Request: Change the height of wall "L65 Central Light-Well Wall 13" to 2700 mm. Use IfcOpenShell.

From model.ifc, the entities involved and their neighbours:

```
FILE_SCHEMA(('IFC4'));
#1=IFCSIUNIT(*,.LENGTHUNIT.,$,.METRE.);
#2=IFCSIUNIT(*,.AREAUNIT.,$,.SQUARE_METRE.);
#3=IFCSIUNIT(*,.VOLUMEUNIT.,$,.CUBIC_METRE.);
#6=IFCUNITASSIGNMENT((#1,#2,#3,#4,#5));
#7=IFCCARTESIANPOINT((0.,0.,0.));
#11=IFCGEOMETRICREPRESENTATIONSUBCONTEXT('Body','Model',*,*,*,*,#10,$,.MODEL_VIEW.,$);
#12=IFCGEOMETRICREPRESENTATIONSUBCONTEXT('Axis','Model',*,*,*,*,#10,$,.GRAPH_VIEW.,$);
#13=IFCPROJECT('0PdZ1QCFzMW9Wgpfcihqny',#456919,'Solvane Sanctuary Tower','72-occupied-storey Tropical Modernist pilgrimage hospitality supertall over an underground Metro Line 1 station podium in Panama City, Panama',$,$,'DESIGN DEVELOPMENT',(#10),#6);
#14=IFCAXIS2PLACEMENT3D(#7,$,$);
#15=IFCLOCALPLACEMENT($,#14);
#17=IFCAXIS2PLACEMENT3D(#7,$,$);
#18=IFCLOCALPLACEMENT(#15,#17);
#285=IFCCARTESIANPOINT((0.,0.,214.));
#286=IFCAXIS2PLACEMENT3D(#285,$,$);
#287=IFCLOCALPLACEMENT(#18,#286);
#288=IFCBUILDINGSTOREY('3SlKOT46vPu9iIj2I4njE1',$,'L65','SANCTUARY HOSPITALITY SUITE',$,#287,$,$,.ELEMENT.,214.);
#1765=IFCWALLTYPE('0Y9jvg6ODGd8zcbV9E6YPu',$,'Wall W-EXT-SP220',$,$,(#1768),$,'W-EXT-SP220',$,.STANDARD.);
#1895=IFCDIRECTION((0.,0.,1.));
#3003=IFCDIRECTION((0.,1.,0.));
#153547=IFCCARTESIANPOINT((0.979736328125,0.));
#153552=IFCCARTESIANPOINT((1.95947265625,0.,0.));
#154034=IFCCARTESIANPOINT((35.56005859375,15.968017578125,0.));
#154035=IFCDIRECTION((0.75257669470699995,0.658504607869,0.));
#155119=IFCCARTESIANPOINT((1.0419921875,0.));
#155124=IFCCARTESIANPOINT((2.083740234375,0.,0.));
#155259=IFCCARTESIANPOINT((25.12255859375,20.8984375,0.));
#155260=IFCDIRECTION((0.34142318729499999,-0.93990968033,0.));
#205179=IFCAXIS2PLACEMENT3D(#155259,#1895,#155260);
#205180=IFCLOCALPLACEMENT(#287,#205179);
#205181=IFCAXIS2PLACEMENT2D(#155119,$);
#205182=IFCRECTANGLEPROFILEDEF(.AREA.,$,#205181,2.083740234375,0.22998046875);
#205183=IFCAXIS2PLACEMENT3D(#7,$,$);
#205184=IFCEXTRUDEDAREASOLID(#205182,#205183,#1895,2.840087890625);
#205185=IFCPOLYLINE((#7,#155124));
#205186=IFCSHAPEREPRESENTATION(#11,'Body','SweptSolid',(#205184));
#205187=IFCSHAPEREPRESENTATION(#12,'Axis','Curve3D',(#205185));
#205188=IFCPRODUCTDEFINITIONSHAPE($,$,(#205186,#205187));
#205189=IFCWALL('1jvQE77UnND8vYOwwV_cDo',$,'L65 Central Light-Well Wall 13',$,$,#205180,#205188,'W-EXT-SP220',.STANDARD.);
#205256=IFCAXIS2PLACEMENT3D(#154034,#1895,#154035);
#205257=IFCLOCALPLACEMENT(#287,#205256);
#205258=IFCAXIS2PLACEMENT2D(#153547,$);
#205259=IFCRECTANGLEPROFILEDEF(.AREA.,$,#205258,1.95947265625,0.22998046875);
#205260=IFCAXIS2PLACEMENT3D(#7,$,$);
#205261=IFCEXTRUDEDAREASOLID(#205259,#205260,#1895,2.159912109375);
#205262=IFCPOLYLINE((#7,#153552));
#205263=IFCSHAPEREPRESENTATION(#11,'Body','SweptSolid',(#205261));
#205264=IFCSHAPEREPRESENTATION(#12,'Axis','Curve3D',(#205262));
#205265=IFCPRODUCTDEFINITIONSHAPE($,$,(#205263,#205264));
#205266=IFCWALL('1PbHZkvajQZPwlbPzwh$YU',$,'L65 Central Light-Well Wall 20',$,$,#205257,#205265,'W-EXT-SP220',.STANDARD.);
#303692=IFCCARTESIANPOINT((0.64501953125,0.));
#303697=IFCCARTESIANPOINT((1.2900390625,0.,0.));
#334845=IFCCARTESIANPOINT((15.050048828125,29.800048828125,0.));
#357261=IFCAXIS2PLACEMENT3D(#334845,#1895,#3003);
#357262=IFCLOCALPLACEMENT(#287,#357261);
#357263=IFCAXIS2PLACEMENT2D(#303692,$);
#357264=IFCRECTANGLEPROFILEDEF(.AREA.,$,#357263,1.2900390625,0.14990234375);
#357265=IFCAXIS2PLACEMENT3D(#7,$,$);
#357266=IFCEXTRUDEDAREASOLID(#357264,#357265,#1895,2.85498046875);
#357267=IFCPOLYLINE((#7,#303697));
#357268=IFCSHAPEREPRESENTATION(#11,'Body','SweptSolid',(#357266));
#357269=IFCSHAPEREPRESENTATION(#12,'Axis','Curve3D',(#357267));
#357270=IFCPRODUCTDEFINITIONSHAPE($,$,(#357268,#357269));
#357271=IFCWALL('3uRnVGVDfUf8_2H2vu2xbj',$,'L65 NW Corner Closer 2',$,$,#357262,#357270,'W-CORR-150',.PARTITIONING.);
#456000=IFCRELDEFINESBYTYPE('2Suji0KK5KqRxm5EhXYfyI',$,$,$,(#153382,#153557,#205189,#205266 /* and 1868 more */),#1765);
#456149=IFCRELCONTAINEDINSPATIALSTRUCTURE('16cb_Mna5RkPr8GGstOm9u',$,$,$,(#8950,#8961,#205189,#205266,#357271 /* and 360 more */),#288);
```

```python
import ifcopenshell
import ifcopenshell.geom
import ifcopenshell.util.representation
import ifcopenshell.util.shape
import ifcopenshell.util.unit

model = ifcopenshell.open("model.ifc")
unit_scale = ifcopenshell.util.unit.calculate_unit_scale(model)
settings = ifcopenshell.geom.settings()


def volume(element):
    """Net volume in cubic metres, openings subtracted."""
    shape = ifcopenshell.geom.create_shape(settings, element)
    return ifcopenshell.util.shape.get_volume(shape.geometry)


wall = model.by_id(205189)
before = volume(wall)

body = ifcopenshell.util.representation.get_representation(wall, "Model", "Body")
solid = body.Items[0]
old_height = solid.Depth
solid.Depth = 2.7 / unit_scale
after = volume(wall)

print(f"height {old_height:g} -> {solid.Depth:g}, volume {before:.3f} -> {after:.3f} m3")

model.write("model_rev.ifc")
```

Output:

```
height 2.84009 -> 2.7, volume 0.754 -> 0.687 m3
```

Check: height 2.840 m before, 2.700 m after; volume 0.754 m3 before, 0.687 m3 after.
